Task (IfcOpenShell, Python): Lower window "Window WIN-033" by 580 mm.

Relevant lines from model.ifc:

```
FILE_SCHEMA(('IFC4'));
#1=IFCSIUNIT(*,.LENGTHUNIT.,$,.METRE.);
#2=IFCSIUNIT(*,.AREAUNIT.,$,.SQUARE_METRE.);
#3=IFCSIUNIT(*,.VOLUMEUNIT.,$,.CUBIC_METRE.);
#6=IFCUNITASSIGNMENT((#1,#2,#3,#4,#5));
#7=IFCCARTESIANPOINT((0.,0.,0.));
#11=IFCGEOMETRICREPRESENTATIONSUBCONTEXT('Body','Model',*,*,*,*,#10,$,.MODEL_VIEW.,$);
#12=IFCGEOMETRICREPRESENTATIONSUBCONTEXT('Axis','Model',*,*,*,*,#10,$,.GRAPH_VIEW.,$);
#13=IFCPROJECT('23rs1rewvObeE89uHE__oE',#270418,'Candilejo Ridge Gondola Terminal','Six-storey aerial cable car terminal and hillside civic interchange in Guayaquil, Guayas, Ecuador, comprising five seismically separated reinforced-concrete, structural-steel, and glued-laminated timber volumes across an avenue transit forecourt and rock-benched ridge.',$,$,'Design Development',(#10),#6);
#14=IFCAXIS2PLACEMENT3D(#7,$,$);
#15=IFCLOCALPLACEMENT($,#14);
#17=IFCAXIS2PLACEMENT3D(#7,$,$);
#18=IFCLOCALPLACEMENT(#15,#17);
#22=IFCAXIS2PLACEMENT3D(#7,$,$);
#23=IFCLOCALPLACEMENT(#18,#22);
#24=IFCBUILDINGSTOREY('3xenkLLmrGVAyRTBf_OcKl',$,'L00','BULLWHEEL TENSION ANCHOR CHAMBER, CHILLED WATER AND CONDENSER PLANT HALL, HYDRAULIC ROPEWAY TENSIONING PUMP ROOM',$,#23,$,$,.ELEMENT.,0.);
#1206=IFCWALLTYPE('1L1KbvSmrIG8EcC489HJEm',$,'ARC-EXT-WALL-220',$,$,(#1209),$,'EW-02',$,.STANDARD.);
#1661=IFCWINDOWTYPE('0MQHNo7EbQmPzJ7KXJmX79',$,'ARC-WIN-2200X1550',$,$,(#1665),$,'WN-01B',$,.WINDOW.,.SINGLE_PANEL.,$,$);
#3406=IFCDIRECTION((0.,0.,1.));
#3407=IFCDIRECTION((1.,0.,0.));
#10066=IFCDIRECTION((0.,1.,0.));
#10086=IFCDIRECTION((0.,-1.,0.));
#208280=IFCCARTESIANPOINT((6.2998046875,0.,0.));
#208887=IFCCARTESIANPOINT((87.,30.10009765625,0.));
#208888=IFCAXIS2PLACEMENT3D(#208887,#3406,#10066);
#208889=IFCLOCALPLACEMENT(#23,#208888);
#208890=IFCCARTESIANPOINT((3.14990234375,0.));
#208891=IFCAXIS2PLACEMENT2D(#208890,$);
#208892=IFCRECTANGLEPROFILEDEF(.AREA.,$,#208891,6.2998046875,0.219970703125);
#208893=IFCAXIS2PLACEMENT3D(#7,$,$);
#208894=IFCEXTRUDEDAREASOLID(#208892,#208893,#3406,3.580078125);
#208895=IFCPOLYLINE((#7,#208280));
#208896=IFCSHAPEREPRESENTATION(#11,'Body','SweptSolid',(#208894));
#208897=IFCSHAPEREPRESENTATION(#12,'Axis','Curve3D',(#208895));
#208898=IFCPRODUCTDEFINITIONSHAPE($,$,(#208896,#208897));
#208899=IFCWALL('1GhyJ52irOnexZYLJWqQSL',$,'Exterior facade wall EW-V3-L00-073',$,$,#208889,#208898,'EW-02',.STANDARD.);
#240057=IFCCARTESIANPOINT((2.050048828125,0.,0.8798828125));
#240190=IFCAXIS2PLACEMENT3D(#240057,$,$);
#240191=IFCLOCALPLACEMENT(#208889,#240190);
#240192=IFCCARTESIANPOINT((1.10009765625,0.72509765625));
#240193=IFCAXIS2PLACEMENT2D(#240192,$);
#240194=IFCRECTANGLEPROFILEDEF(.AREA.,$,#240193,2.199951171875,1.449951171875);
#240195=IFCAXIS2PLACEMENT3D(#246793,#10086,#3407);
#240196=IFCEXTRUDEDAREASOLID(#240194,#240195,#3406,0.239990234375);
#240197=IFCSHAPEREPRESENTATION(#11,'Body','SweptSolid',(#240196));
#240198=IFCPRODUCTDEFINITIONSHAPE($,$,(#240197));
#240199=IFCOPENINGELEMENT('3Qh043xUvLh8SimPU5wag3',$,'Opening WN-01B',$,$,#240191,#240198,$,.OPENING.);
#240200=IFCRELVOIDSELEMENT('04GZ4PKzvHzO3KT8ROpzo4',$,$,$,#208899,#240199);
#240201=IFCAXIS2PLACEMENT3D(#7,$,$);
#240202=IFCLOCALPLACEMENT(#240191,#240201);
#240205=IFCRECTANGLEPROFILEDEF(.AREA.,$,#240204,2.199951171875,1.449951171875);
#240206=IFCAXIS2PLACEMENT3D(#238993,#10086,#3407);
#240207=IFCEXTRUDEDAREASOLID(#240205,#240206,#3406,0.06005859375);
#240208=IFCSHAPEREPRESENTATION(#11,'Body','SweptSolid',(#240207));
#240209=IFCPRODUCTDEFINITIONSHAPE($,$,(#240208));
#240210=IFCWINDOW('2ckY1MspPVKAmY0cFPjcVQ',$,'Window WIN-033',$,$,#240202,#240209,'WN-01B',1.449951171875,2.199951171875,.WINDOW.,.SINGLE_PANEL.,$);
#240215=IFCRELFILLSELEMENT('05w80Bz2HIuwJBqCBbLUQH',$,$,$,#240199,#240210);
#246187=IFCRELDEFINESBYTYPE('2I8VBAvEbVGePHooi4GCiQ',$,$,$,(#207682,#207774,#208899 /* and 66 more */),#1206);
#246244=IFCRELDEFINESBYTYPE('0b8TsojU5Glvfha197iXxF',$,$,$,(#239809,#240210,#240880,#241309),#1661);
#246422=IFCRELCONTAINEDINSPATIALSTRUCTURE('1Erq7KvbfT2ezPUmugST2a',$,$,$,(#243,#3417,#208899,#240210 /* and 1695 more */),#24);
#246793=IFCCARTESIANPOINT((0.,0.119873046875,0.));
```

```python
import numpy as np
import ifcopenshell
import ifcopenshell.api.geometry
import ifcopenshell.util.placement
import ifcopenshell.util.unit

model = ifcopenshell.open("model.ifc")
unit_scale = ifcopenshell.util.unit.calculate_unit_scale(model)

window = model.by_guid("2ckY1MspPVKAmY0cFPjcVQ")
opening = window.FillsVoids[0].RelatingOpeningElement
dz = -0.58

shift = np.array([0.0, 0.0, dz])
# The window is placed relative to its opening, so it follows when the opening moves.
matrix = ifcopenshell.util.placement.get_local_placement(opening.ObjectPlacement)
matrix[:3, 3] += shift
ifcopenshell.api.geometry.edit_object_placement(
    model, product=opening, matrix=matrix, is_si=False, should_transform_children=True
)

print(f"moved by {dz * unit_scale:+.3f} m")

model.write("model_rev.ifc")
```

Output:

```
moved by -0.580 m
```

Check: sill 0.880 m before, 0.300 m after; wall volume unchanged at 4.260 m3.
